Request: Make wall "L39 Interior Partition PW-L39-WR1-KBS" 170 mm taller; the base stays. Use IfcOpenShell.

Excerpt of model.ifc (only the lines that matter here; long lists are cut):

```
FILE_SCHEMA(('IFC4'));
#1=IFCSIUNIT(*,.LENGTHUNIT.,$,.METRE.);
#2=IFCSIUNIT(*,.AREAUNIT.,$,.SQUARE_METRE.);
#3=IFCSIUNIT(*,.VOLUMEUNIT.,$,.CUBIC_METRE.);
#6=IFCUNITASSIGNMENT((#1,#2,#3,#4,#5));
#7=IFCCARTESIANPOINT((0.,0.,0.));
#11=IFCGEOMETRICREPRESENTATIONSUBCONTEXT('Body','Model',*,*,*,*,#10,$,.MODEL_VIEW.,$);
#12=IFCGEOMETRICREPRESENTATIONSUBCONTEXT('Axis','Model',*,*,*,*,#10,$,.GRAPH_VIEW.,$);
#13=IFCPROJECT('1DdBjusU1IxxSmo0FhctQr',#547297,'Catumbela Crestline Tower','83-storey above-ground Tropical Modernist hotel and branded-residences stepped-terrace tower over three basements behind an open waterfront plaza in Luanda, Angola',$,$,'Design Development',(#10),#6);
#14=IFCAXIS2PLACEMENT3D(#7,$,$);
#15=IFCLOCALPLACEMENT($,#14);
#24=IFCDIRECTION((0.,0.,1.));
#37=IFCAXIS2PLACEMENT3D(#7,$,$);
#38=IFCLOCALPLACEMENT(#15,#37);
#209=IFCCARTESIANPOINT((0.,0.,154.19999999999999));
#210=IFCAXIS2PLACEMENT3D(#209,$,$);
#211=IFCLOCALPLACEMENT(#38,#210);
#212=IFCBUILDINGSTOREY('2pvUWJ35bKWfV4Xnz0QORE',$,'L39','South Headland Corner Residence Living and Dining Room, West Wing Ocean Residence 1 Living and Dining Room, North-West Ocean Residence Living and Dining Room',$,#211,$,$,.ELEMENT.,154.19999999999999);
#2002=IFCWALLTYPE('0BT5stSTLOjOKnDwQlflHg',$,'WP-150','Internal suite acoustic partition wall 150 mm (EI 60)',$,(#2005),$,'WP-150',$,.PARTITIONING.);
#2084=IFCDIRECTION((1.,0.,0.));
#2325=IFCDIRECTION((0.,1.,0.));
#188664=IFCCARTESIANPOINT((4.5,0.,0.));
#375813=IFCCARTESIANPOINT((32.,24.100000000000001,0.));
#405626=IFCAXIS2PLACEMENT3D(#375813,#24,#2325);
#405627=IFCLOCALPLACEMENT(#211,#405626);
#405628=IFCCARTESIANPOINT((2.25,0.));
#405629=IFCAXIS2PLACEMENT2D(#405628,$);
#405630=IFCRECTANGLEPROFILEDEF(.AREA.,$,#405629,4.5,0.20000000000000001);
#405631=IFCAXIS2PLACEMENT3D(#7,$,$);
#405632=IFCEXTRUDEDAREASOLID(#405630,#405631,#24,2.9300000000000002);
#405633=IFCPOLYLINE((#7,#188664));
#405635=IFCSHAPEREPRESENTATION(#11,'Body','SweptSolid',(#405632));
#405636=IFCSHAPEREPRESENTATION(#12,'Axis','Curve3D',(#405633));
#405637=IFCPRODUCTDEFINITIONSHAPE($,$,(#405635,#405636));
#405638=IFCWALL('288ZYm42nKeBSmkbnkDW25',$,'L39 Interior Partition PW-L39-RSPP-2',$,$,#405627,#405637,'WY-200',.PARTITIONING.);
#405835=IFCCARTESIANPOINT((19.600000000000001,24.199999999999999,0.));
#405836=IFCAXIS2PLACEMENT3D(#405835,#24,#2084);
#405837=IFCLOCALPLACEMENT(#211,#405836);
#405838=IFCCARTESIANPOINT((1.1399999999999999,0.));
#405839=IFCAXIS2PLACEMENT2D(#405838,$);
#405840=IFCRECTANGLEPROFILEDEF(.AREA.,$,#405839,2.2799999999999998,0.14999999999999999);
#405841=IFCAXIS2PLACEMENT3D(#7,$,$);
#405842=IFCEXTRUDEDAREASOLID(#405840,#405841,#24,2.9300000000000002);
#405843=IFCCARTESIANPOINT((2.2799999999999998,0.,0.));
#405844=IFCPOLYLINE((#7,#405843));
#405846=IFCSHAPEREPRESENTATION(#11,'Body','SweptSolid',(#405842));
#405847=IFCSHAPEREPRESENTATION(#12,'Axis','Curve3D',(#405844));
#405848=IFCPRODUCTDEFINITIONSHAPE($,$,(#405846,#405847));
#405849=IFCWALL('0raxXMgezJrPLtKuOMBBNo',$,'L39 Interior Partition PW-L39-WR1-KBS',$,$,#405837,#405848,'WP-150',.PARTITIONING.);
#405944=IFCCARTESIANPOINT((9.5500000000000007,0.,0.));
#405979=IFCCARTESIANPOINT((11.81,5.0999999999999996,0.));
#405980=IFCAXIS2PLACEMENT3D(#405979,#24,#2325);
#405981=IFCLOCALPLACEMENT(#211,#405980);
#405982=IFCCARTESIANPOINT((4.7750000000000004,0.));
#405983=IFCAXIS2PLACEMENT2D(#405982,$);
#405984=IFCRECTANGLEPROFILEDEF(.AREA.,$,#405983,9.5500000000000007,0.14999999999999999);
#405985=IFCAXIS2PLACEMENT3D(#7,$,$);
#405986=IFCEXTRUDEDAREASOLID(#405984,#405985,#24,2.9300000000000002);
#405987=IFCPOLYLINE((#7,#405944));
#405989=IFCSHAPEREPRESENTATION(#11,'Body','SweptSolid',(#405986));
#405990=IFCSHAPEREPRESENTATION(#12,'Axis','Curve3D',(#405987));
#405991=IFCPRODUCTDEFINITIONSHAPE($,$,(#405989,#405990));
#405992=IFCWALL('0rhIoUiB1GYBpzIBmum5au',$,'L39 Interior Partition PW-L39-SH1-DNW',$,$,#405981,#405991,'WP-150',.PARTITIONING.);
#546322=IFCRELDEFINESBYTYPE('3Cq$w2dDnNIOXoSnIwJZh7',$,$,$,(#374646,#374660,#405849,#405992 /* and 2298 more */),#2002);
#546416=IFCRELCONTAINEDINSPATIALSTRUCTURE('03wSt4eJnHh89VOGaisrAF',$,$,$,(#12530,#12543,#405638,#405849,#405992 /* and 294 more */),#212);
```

```python
import ifcopenshell
import ifcopenshell.geom
import ifcopenshell.util.representation
import ifcopenshell.util.shape
import ifcopenshell.util.unit

model = ifcopenshell.open("model.ifc")
unit_scale = ifcopenshell.util.unit.calculate_unit_scale(model)
settings = ifcopenshell.geom.settings()


def volume(element):
    """Net volume in cubic metres, openings subtracted."""
    shape = ifcopenshell.geom.create_shape(settings, element)
    return ifcopenshell.util.shape.get_volume(shape.geometry)


wall = model.by_id(405849)
before = volume(wall)

body = ifcopenshell.util.representation.get_representation(wall, "Model", "Body")
solid = body.Items[0]
old_height = solid.Depth
solid.Depth += 0.17 / unit_scale
after = volume(wall)

print(f"height {old_height:g} -> {solid.Depth:g}, volume {before:.3f} -> {after:.3f} m3")

model.write("model_rev.ifc")
```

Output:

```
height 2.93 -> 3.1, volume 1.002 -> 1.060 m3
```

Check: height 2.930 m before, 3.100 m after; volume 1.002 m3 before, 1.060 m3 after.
